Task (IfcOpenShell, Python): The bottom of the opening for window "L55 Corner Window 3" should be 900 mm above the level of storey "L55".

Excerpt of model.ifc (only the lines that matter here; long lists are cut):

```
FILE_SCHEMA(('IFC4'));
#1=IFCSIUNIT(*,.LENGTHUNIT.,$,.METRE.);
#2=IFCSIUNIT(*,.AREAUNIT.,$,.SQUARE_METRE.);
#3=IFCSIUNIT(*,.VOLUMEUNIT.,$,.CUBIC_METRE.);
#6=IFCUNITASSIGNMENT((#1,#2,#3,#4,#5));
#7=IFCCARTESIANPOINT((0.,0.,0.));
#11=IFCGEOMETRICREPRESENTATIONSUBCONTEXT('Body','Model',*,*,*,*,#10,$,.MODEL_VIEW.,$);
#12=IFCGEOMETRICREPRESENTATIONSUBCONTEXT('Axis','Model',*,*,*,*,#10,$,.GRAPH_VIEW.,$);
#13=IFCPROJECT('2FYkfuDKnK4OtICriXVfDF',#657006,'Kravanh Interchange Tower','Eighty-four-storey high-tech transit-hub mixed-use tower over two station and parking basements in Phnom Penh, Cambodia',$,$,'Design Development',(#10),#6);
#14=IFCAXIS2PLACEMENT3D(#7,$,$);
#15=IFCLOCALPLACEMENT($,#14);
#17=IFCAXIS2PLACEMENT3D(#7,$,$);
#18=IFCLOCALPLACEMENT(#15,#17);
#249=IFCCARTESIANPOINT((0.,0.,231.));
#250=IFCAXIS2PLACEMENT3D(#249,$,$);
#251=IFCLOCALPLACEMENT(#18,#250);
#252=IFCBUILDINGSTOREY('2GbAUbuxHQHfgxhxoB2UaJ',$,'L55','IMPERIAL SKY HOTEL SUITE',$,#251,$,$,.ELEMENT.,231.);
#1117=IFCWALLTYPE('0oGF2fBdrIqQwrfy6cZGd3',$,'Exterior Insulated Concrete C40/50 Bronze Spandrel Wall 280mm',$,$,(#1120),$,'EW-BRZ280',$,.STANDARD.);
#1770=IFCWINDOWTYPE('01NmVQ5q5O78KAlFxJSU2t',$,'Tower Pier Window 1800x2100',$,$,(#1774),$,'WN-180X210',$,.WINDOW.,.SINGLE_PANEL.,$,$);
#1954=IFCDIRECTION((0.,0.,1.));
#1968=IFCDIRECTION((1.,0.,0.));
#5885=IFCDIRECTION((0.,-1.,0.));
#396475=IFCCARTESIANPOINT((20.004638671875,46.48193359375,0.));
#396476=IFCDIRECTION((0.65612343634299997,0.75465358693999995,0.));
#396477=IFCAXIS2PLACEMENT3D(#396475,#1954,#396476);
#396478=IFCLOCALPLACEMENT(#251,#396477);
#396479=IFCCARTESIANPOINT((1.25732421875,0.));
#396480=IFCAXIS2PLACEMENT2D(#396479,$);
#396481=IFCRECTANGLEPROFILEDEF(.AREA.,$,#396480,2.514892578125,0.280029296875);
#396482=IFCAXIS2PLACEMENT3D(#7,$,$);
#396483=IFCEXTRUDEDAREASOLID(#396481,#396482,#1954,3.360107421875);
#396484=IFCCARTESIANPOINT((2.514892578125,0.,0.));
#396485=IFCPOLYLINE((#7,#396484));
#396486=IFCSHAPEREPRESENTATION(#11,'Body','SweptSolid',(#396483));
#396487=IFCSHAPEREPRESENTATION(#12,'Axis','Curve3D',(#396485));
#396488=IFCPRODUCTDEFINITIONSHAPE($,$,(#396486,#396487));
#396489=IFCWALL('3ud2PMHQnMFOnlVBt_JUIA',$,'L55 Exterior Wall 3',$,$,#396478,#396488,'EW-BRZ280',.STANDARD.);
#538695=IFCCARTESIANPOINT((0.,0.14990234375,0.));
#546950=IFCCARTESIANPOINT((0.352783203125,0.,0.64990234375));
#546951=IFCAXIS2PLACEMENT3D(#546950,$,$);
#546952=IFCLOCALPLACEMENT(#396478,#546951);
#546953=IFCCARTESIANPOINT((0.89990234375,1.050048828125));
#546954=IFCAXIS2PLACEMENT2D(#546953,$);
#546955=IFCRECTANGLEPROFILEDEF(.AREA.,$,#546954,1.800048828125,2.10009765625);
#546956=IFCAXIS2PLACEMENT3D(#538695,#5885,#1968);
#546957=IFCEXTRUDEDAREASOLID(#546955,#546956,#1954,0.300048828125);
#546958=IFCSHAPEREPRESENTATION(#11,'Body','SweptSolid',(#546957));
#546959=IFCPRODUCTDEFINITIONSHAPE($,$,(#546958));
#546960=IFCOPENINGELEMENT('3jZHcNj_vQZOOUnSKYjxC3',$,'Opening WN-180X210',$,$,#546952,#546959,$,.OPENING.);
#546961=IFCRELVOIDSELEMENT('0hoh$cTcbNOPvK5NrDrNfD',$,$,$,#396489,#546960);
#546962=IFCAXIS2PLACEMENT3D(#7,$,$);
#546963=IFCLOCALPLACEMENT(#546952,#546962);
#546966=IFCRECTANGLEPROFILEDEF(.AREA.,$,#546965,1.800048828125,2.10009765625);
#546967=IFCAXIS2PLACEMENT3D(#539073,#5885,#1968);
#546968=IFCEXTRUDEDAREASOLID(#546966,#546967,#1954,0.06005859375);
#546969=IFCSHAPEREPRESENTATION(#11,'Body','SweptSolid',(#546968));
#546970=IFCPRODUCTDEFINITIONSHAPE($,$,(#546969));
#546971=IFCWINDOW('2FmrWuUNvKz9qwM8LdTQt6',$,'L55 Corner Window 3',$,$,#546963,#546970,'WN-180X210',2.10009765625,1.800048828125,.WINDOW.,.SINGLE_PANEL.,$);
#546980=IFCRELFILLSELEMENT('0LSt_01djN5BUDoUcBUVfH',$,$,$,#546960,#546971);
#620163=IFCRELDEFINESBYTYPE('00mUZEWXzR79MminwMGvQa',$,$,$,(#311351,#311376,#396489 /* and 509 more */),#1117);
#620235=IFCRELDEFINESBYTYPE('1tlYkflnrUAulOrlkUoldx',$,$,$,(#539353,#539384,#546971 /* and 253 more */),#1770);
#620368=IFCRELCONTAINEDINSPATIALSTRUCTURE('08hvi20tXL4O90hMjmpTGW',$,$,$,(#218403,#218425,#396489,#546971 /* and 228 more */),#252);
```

```python
import numpy as np
import ifcopenshell
import ifcopenshell.api.geometry
import ifcopenshell.geom
import ifcopenshell.util.element
import ifcopenshell.util.placement
import ifcopenshell.util.shape
import ifcopenshell.util.unit

model = ifcopenshell.open("model.ifc")
unit_scale = ifcopenshell.util.unit.calculate_unit_scale(model)

window = model.by_guid("2FmrWuUNvKz9qwM8LdTQt6")
opening = window.FillsVoids[0].RelatingOpeningElement
storey = ifcopenshell.util.element.get_container(window, ifc_class="IfcBuildingStorey")
level = ifcopenshell.util.placement.get_local_placement(storey.ObjectPlacement)[2, 3]

# The opening's origin need not be at the sill, so measure its lowest point.
shape = ifcopenshell.geom.create_shape(ifcopenshell.geom.settings(), opening)
bottom = ifcopenshell.util.shape.get_shape_bottom_elevation(shape, shape.geometry) / unit_scale
dz = level + 0.9 / unit_scale - bottom

shift = np.array([0.0, 0.0, dz])
# The window is placed relative to its opening, so it follows when the opening moves.
matrix = ifcopenshell.util.placement.get_local_placement(opening.ObjectPlacement)
matrix[:3, 3] += shift
ifcopenshell.api.geometry.edit_object_placement(
    model, product=opening, matrix=matrix, is_si=False, should_transform_children=True
)

print(f"moved by {dz * unit_scale:+.3f} m")

model.write("model_v2.ifc")
```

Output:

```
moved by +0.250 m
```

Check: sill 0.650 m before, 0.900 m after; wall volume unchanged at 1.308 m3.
